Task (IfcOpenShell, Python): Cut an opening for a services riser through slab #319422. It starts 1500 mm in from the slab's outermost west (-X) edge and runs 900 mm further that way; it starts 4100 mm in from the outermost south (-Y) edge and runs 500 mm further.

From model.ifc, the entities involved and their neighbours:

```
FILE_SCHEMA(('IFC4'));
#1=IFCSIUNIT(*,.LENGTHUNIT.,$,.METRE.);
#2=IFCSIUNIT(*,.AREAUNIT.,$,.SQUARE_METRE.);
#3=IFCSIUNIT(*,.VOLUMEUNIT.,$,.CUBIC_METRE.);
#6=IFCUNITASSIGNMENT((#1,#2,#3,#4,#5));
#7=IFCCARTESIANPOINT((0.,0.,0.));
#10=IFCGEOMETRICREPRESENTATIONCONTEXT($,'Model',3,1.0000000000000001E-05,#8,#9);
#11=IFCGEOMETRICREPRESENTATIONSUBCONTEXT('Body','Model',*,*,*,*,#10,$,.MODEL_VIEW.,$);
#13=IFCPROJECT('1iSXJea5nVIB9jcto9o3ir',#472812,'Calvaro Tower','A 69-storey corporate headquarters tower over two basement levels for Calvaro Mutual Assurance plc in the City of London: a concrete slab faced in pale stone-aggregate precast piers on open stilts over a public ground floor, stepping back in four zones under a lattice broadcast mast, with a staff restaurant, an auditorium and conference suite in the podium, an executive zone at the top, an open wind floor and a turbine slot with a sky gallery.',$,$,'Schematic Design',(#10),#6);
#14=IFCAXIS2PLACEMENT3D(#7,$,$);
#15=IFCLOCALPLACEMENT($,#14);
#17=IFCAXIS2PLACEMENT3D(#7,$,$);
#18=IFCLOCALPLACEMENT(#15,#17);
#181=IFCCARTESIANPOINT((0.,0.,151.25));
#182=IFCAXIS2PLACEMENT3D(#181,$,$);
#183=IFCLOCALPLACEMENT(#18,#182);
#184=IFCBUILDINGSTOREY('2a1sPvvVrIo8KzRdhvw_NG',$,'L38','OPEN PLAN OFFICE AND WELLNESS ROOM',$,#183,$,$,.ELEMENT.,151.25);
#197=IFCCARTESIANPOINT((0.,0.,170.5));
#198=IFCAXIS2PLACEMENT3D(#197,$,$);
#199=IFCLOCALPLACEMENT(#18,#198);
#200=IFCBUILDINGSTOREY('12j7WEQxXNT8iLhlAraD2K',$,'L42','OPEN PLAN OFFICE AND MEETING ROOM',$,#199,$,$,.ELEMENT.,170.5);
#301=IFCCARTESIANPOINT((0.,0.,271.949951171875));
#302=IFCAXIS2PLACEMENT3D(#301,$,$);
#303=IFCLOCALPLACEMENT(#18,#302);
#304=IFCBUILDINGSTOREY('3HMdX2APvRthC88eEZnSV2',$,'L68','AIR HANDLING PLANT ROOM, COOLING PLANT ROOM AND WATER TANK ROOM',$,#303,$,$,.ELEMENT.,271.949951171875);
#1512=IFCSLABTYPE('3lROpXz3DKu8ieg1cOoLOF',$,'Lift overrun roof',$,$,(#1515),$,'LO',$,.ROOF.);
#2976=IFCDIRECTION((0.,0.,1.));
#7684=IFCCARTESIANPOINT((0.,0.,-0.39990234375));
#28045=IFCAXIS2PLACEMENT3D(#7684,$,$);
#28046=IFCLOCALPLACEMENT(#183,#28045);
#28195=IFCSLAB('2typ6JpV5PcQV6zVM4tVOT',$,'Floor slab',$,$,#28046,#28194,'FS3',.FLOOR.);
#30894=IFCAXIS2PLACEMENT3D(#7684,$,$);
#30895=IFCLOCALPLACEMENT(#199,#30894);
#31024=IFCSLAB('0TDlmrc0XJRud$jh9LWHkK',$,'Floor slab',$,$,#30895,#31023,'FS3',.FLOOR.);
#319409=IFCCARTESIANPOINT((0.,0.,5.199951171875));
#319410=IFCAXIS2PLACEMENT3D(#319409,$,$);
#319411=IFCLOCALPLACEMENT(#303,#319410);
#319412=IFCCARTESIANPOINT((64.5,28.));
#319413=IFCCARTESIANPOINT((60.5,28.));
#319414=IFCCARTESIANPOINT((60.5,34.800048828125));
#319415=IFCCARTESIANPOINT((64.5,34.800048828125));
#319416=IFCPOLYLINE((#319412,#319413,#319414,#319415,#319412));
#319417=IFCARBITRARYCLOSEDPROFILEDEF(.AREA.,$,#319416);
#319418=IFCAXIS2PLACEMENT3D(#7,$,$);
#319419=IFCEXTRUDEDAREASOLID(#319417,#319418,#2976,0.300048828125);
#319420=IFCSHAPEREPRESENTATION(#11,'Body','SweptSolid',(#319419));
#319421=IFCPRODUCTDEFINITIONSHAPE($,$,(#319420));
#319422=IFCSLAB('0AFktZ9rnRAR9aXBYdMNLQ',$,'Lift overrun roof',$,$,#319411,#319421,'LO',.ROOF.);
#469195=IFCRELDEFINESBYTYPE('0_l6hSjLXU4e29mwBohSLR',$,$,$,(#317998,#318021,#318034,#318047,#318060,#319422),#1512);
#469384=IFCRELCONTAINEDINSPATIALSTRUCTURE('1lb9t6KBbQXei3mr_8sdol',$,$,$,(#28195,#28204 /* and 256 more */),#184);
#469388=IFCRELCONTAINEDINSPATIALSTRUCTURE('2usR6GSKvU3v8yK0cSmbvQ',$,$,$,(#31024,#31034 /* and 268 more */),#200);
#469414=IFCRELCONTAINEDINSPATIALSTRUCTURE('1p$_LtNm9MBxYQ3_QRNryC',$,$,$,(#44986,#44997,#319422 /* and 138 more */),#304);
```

```python
import numpy as np
import ifcopenshell
import ifcopenshell.api.feature
import ifcopenshell.api.geometry
import ifcopenshell.api.root
import ifcopenshell.geom
import ifcopenshell.util.placement
import ifcopenshell.util.representation
import ifcopenshell.util.shape
import ifcopenshell.util.unit

model = ifcopenshell.open("model.ifc")
unit_scale = ifcopenshell.util.unit.calculate_unit_scale(model)
settings = ifcopenshell.geom.settings()


def volume(element):
    """Net volume in cubic metres, openings subtracted."""
    shape = ifcopenshell.geom.create_shape(settings, element)
    return ifcopenshell.util.shape.get_volume(shape.geometry)


slab = model.by_guid("0AFktZ9rnRAR9aXBYdMNLQ")
before = volume(slab)

# Extent in the slab's own axes, in metres. The edges named are its -X and -Y sides.
slab_shape = ifcopenshell.geom.create_shape(settings, slab)
vertices = ifcopenshell.util.shape.get_vertices(slab_shape.geometry)
x_min, y_min, bottom = vertices.min(axis=0)
top = vertices[:, 2].max()

opening = ifcopenshell.api.root.create_entity(model, ifc_class="IfcOpeningElement", name="Services riser opening", predefined_type="OPENING")
context = ifcopenshell.util.representation.get_context(model, "Model", "Body", "MODEL_VIEW")
width, depth = 0.9, 0.5
outline = [(0.0, 0.0), (width, 0.0), (width, depth), (0.0, depth), (0.0, 0.0)]
# Overshoot both faces by 50 mm so the cut is clean.
shape = ifcopenshell.api.geometry.add_slab_representation(
    model, context=context, depth=top - bottom + 0.1, polyline=outline
)
ifcopenshell.api.geometry.assign_representation(model, product=opening, representation=shape)

matrix = ifcopenshell.util.placement.get_local_placement(slab.ObjectPlacement)
matrix[:, 3] = matrix @ np.append(np.array([x_min + 1.5, y_min + 4.1, bottom - 0.05]) / unit_scale, 1.0)
ifcopenshell.api.geometry.edit_object_placement(model, product=opening, matrix=matrix, is_si=False)
ifcopenshell.api.feature.add_feature(model, feature=opening, element=slab)

after = volume(slab)

print(f"slab volume {before:.3f} -> {after:.3f} m3")

model.write("model_updated.ifc")
```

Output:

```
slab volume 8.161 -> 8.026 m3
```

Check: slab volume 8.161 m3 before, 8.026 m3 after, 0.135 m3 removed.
